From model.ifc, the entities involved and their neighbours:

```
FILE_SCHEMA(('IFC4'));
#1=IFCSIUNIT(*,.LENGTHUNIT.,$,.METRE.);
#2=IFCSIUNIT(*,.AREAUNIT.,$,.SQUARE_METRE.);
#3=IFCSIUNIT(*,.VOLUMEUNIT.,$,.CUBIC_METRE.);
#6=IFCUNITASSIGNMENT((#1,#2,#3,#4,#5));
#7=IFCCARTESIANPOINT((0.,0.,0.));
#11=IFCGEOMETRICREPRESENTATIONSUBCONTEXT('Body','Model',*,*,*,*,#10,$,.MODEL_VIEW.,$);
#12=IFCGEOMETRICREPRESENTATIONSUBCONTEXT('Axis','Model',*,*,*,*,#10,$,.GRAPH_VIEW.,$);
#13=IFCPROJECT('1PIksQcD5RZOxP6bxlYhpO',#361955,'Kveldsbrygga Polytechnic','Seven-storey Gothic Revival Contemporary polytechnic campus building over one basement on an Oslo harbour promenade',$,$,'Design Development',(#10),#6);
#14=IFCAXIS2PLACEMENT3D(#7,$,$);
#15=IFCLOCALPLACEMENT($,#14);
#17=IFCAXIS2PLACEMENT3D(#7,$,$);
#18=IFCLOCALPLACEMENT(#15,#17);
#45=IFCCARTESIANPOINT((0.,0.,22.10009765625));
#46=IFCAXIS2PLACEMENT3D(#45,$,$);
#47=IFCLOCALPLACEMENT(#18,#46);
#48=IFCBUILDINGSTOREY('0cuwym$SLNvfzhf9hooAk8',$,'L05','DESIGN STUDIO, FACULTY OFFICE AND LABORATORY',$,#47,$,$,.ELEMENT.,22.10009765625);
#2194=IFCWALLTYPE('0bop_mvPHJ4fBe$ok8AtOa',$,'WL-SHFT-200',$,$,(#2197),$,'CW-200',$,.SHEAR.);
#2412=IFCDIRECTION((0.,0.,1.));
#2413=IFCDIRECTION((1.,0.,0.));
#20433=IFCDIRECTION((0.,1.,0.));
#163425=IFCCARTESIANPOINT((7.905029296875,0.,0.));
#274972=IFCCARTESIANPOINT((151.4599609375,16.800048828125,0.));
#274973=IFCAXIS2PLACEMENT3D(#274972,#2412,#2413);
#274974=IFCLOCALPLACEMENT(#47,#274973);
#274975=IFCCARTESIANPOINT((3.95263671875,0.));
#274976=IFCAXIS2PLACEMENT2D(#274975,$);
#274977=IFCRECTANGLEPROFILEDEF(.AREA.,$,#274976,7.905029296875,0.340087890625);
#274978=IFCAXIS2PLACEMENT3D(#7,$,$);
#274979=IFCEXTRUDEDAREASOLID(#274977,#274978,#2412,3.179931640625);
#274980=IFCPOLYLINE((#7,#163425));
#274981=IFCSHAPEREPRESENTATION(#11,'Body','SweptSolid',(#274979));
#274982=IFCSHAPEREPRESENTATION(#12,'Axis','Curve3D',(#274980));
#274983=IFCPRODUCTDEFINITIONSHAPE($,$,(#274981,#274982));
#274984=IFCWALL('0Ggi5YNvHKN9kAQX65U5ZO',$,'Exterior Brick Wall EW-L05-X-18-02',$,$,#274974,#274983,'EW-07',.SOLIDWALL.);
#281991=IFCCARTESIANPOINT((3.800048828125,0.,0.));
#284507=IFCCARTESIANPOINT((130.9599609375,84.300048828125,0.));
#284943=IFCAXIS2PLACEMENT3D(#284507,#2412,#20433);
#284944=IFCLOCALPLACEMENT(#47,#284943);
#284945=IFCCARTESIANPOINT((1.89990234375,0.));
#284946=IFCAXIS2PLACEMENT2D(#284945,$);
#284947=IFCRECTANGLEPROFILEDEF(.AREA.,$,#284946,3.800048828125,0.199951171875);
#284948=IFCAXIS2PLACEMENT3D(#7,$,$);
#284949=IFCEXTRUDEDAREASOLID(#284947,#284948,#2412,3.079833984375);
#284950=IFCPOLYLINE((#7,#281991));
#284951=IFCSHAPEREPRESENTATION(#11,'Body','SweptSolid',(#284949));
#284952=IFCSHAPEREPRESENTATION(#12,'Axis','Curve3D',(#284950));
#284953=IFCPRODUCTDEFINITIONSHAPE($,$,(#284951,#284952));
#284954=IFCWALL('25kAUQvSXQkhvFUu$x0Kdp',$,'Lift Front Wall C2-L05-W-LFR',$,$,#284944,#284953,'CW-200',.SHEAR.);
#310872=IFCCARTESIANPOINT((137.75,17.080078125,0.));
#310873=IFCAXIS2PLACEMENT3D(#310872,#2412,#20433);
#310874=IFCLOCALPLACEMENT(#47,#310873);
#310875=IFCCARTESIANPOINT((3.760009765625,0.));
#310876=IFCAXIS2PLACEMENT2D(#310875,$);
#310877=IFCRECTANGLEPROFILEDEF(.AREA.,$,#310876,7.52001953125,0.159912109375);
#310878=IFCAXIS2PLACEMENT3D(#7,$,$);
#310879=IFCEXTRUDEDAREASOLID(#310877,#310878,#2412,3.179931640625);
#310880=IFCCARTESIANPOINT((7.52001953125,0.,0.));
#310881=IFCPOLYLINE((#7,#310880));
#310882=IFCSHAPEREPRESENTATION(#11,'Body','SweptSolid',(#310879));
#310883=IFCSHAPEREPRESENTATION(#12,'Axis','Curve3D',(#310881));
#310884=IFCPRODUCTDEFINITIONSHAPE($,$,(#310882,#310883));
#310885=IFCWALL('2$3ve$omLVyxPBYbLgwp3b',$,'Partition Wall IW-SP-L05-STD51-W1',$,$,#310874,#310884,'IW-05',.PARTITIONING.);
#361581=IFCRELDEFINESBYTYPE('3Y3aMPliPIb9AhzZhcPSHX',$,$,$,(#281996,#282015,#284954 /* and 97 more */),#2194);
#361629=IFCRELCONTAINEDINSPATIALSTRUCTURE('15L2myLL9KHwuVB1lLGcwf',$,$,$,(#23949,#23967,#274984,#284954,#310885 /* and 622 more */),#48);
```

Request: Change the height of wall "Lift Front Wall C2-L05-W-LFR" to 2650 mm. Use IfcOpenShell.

```python
import ifcopenshell
import ifcopenshell.geom
import ifcopenshell.util.representation
import ifcopenshell.util.shape
import ifcopenshell.util.unit

model = ifcopenshell.open("model.ifc")
unit_scale = ifcopenshell.util.unit.calculate_unit_scale(model)
settings = ifcopenshell.geom.settings()


def volume(element):
    """Net volume in cubic metres, openings subtracted."""
    shape = ifcopenshell.geom.create_shape(settings, element)
    return ifcopenshell.util.shape.get_volume(shape.geometry)


wall = model.by_guid("25kAUQvSXQkhvFUu$x0Kdp")
before = volume(wall)

body = ifcopenshell.util.representation.get_representation(wall, "Model", "Body")
solid = body.Items[0]
old_height = solid.Depth
solid.Depth = 2.65 / unit_scale
after = volume(wall)

print(f"height {old_height:g} -> {solid.Depth:g}, volume {before:.3f} -> {after:.3f} m3")

model.write("model_v2.ifc")
```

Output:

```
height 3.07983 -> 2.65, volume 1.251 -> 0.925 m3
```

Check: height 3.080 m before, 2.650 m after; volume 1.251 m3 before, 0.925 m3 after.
